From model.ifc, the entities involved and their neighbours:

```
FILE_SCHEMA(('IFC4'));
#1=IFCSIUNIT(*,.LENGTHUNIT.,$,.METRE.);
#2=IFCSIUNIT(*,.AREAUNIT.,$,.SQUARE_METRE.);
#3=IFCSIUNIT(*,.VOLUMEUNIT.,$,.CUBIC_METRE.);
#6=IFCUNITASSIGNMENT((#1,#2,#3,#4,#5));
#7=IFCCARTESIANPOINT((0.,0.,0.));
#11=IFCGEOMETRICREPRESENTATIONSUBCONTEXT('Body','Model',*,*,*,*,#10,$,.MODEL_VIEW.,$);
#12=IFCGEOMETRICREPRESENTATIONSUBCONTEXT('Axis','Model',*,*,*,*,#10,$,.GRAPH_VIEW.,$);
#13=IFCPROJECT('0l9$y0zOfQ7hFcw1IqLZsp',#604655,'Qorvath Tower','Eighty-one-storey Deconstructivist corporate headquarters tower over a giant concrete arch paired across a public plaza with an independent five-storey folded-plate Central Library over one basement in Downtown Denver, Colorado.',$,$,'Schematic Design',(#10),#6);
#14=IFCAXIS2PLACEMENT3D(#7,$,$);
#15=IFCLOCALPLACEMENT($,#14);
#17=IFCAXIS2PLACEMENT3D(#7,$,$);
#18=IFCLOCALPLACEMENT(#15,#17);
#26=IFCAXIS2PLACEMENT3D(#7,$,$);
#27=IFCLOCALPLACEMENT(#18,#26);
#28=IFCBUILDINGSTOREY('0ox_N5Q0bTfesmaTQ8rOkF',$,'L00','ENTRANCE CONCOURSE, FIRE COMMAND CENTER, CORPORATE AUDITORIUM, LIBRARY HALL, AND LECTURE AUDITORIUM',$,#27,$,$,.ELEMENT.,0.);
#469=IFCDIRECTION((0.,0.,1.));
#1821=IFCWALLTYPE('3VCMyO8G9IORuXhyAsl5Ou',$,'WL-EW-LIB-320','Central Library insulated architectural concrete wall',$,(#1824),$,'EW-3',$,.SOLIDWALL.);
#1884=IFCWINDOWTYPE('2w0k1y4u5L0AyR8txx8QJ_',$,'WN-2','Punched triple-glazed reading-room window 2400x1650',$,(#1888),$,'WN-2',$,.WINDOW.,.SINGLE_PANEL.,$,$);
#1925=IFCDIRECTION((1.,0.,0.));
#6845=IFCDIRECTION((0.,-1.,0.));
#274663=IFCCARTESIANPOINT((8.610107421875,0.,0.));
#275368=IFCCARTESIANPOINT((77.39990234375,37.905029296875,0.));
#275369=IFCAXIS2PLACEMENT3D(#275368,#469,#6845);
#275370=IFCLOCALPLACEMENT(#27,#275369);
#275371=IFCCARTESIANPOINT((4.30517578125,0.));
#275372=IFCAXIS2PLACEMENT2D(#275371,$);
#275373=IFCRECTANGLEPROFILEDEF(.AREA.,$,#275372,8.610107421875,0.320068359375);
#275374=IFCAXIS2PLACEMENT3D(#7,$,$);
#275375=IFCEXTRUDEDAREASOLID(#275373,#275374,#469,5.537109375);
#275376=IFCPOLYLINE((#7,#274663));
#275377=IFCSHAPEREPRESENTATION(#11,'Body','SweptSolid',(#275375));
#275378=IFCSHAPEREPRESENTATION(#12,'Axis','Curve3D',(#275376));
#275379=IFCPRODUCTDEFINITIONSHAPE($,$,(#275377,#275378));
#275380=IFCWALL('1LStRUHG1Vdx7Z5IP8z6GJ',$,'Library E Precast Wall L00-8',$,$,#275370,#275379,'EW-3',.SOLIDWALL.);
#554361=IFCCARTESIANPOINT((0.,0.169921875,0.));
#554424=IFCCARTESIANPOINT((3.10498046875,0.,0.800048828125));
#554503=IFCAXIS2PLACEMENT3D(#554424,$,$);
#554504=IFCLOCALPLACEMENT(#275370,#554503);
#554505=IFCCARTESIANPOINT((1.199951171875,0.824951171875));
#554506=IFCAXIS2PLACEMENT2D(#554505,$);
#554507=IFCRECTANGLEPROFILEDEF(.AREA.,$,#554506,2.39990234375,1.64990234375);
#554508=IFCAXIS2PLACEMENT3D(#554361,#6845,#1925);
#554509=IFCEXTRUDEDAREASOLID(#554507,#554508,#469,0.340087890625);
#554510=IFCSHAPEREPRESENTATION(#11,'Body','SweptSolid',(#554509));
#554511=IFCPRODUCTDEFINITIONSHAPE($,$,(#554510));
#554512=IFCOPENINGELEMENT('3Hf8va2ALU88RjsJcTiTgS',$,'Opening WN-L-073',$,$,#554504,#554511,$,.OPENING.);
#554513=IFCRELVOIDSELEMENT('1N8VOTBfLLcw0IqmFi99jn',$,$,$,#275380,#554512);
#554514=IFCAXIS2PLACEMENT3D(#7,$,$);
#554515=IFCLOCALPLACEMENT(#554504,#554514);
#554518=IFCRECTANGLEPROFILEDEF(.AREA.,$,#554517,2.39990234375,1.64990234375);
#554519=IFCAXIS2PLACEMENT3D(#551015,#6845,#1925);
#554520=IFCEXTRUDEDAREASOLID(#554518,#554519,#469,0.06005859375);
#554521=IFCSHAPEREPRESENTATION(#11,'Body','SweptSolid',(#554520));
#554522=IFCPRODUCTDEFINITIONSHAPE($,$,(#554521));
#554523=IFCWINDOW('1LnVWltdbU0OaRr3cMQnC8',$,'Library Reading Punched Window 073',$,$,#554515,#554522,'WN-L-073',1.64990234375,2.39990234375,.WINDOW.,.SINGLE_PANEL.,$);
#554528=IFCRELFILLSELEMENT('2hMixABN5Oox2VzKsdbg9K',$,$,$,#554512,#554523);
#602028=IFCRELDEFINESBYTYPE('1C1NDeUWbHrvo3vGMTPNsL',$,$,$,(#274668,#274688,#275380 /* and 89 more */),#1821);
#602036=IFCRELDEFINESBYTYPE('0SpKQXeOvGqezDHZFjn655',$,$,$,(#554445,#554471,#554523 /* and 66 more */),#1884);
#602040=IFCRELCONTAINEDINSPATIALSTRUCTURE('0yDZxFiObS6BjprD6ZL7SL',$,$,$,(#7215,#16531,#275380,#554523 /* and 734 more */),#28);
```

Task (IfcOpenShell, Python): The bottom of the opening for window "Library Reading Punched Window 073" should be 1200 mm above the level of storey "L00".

```python
import numpy as np
import ifcopenshell
import ifcopenshell.api.geometry
import ifcopenshell.geom
import ifcopenshell.util.element
import ifcopenshell.util.placement
import ifcopenshell.util.shape
import ifcopenshell.util.unit

model = ifcopenshell.open("model.ifc")
unit_scale = ifcopenshell.util.unit.calculate_unit_scale(model)

window = model.by_id(554523)
opening = window.FillsVoids[0].RelatingOpeningElement
storey = ifcopenshell.util.element.get_container(window, ifc_class="IfcBuildingStorey")
level = ifcopenshell.util.placement.get_local_placement(storey.ObjectPlacement)[2, 3]

# The opening's origin need not be at the sill, so measure its lowest point.
shape = ifcopenshell.geom.create_shape(ifcopenshell.geom.settings(), opening)
bottom = ifcopenshell.util.shape.get_shape_bottom_elevation(shape, shape.geometry) / unit_scale
dz = level + 1.2 / unit_scale - bottom

shift = np.array([0.0, 0.0, dz])
# The window is placed relative to its opening, so it follows when the opening moves.
matrix = ifcopenshell.util.placement.get_local_placement(opening.ObjectPlacement)
matrix[:3, 3] += shift
ifcopenshell.api.geometry.edit_object_placement(
    model, product=opening, matrix=matrix, is_si=False, should_transform_children=True
)

print(f"moved by {dz * unit_scale:+.3f} m")

model.write("model_edited.ifc")
```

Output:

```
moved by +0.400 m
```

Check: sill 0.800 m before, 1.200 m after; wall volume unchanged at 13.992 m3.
